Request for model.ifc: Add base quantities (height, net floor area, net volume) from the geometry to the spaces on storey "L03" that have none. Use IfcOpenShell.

First a look at what the model holds.

```python
import ifcopenshell
import ifcopenshell.util.element
import ifcopenshell.util.unit

model = ifcopenshell.open("model.ifc")
print(model.schema)
for unit_type in ("LENGTHUNIT", "AREAUNIT", "VOLUMEUNIT"):
    print(unit_type, ifcopenshell.util.unit.calculate_unit_scale(model, unit_type))
storey = next(s for s in model.by_type("IfcBuildingStorey") if s.Name == "L03")
spaces = [e for e in ifcopenshell.util.element.get_decomposition(storey) if e.is_a("IfcSpace")]
for e in sorted(spaces, key=lambda e: e.id()):
    print(e.id(), e.is_a(), e.Name, list(ifcopenshell.util.element.get_psets(e, qtos_only=True)), sep=" | ")
```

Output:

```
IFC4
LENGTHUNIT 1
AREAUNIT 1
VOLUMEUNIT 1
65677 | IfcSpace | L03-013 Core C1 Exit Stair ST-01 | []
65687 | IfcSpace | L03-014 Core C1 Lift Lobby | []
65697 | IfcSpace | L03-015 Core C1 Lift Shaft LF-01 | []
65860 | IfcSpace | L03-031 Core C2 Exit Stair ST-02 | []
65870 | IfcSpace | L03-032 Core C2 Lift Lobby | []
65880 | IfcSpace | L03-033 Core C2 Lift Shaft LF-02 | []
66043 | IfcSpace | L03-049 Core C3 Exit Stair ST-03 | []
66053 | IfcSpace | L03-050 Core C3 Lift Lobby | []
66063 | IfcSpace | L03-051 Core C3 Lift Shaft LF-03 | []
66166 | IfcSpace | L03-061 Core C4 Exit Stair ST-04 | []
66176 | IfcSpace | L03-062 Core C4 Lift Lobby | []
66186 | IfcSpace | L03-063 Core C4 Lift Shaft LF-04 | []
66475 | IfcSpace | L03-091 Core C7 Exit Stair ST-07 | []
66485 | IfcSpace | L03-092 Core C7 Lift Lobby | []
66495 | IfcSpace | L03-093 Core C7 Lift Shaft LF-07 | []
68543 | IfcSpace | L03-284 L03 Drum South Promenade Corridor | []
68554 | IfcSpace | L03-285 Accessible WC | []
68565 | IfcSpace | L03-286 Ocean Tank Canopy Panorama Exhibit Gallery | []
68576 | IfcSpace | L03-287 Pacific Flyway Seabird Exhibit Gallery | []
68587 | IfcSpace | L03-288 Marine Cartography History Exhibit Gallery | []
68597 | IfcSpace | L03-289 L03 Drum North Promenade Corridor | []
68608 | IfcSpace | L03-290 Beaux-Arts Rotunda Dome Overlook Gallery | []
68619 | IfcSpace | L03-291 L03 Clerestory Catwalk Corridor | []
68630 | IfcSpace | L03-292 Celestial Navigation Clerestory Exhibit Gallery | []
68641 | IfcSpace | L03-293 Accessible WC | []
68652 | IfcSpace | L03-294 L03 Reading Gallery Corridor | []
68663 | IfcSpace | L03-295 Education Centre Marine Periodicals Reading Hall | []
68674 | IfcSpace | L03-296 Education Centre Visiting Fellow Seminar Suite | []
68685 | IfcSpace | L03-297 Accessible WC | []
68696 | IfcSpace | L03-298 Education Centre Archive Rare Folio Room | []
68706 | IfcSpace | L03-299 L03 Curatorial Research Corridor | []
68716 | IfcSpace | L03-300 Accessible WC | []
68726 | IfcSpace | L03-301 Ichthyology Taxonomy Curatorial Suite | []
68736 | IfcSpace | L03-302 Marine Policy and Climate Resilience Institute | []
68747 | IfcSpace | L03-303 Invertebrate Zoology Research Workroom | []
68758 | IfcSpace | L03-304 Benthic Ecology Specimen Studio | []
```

```python
import ifcopenshell
import ifcopenshell.api.pset
import ifcopenshell.geom
import ifcopenshell.util.element
import ifcopenshell.util.shape
import ifcopenshell.util.unit

model = ifcopenshell.open("model.ifc")
unit_scale = ifcopenshell.util.unit.calculate_unit_scale(model)
area_scale = ifcopenshell.util.unit.calculate_unit_scale(model, "AREAUNIT")
volume_scale = ifcopenshell.util.unit.calculate_unit_scale(model, "VOLUMEUNIT")
settings = ifcopenshell.geom.settings()

storey = next(s for s in model.by_type("IfcBuildingStorey") if s.Name == "L03")
spaces = [e for e in ifcopenshell.util.element.get_decomposition(storey) if e.is_a("IfcSpace")]

for e in sorted(spaces, key=lambda e: e.id()):
    if ifcopenshell.util.element.get_psets(e, qtos_only=True, should_inherit=False):
        continue
    # Geometry comes back in metres, in the element's own axes.
    shape = ifcopenshell.geom.create_shape(settings, e)
    values = {
        "Height": ifcopenshell.util.shape.get_z(shape.geometry) / unit_scale,
        "NetFloorArea": ifcopenshell.util.shape.get_footprint_area(shape.geometry) / area_scale,
        "NetVolume": ifcopenshell.util.shape.get_volume(shape.geometry) / volume_scale,
    }
    qto = ifcopenshell.api.pset.add_qto(model, product=e, name="Qto_SpaceBaseQuantities")
    ifcopenshell.api.pset.edit_qto(model, qto=qto, properties=values)
    print(e.id(), {k: round(v, 3) for k, v in values.items()})

model.write("model_updated.ifc")
```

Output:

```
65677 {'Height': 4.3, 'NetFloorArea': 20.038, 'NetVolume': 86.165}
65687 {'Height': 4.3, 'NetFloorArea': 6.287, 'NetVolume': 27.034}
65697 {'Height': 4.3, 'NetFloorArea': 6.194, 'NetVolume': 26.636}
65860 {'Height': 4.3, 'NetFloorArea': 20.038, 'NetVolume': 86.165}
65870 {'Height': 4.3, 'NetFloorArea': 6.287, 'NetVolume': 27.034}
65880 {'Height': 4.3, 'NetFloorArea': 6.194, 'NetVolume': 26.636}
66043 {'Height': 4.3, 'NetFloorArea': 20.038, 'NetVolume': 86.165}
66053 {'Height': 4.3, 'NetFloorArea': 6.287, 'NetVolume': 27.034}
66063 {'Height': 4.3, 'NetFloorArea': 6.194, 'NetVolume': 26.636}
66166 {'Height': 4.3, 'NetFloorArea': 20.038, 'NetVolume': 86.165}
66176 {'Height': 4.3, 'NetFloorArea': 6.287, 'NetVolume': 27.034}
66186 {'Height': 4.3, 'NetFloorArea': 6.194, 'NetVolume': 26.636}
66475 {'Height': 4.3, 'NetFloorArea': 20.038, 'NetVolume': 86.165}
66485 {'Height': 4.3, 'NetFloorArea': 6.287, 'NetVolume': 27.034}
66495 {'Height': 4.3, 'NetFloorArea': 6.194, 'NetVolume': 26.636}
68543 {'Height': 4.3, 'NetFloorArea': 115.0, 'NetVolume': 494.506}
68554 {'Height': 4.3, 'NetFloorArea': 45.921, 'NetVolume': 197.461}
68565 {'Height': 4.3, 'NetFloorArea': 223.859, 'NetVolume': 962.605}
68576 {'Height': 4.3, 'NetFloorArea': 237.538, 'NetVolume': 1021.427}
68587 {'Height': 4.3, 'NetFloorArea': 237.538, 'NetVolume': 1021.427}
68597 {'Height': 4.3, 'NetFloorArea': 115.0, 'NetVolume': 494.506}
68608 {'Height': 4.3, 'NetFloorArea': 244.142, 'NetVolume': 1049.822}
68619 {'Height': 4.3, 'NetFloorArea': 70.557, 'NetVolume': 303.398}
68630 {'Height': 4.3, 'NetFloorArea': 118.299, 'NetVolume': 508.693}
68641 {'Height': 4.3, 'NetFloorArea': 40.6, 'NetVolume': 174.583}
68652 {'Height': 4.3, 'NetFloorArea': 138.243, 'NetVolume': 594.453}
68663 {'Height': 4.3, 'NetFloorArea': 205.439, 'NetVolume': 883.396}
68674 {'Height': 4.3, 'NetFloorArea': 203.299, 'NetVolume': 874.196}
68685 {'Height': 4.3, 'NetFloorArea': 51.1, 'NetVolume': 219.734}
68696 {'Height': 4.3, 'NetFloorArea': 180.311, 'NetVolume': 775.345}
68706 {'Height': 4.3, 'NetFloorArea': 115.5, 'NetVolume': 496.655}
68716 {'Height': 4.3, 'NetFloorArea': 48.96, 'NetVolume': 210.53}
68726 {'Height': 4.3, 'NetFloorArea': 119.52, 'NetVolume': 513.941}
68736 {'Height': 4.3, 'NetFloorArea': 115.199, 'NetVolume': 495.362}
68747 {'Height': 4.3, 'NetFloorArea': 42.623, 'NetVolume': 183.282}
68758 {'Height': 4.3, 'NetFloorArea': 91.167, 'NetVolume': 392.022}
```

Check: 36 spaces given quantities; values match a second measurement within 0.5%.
